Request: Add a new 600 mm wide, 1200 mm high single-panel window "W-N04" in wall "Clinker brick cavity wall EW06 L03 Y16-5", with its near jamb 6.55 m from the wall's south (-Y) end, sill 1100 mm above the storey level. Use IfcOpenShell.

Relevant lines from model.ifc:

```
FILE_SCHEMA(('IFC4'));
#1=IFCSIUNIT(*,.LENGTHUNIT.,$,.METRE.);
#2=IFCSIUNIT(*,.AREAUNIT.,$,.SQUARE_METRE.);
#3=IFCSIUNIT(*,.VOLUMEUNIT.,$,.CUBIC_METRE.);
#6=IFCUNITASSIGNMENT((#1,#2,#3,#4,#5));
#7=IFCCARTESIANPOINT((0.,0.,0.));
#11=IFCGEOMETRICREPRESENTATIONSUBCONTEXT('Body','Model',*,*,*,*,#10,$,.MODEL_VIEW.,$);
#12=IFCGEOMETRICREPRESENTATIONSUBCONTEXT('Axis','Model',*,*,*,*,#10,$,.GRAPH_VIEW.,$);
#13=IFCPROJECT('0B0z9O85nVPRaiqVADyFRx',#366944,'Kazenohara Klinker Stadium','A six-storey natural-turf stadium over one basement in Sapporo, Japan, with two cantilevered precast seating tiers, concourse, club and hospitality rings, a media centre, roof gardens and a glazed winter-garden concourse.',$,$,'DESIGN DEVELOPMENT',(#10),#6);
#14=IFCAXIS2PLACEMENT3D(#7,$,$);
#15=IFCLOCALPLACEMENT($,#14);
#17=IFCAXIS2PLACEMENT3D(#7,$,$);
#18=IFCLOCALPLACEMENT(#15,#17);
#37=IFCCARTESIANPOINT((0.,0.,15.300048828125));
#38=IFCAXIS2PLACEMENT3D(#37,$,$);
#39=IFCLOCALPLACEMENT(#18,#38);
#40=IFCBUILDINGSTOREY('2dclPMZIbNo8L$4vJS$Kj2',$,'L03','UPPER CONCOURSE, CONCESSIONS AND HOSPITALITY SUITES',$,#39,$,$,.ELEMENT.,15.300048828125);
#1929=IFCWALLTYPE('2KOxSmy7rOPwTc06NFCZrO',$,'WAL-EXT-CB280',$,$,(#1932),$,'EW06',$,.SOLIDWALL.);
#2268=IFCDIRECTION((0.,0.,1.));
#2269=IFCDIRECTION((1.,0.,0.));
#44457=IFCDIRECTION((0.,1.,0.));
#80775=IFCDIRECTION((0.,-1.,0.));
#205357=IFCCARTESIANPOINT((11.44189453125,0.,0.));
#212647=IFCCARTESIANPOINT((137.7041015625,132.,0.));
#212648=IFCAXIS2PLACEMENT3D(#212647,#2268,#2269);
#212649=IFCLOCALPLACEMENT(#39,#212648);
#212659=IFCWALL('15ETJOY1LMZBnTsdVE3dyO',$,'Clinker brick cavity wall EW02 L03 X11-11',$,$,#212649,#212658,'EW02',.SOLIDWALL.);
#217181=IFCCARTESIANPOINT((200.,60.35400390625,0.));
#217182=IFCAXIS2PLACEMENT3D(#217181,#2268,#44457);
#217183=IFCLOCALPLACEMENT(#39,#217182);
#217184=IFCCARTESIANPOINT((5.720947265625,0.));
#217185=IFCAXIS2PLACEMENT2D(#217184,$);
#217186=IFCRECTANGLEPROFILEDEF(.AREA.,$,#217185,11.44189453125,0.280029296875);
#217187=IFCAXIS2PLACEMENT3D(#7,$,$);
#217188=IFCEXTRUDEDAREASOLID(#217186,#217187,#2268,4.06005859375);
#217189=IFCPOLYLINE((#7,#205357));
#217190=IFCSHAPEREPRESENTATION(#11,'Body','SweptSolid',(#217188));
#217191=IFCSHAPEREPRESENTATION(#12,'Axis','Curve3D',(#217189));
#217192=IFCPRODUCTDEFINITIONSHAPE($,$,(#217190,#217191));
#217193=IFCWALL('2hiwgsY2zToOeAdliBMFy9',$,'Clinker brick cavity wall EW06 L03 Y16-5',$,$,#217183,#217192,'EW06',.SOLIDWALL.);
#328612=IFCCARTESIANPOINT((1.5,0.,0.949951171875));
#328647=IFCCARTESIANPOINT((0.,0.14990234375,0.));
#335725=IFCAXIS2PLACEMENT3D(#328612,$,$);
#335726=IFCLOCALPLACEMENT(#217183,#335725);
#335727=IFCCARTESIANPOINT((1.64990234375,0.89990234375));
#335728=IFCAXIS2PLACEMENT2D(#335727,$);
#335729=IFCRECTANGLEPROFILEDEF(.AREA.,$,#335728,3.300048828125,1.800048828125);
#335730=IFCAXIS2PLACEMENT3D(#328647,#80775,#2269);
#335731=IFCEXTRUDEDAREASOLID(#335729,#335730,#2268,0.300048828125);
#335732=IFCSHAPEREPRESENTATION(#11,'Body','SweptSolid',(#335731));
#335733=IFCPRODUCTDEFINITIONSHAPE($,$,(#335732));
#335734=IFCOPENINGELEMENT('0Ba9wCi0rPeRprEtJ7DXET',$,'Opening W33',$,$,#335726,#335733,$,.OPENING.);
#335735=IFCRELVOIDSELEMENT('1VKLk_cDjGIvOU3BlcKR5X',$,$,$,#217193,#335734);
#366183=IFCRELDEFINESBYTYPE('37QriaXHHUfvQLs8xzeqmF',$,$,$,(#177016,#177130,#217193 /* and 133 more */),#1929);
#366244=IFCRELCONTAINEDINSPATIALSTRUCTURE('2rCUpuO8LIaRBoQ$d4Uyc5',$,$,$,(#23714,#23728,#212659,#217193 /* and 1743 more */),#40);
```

```python
import numpy as np
import ifcopenshell
import ifcopenshell.api.feature
import ifcopenshell.api.geometry
import ifcopenshell.api.root
import ifcopenshell.api.spatial
import ifcopenshell.geom
import ifcopenshell.util.element
import ifcopenshell.util.placement
import ifcopenshell.util.representation
import ifcopenshell.util.shape
import ifcopenshell.util.unit

model = ifcopenshell.open("model.ifc")
unit_scale = ifcopenshell.util.unit.calculate_unit_scale(model)
settings = ifcopenshell.geom.settings()


def volume(element):
    """Net volume in cubic metres, openings subtracted."""
    shape = ifcopenshell.geom.create_shape(settings, element)
    return ifcopenshell.util.shape.get_volume(shape.geometry)


wall = model.by_guid("2hiwgsY2zToOeAdliBMFy9")
storey = ifcopenshell.util.element.get_container(wall, ifc_class="IfcBuildingStorey")
context = ifcopenshell.util.representation.get_context(model, "Model", "Body", "MODEL_VIEW")
before = volume(wall)

width, height, from_end, sill = 0.6, 1.2, 6.55, 1.1  # metres

# The wall runs along its own X axis, and the end named is its -X end.
wall_shape = ifcopenshell.geom.create_shape(settings, wall)
x, y, z = ifcopenshell.util.shape.get_vertices(wall_shape.geometry).T
start = x.min() + from_end
face, thickness = float(y.min()), float(y.max() - y.min())
wall_matrix = ifcopenshell.util.placement.get_local_placement(wall.ObjectPlacement)
level = ifcopenshell.util.placement.get_local_placement(storey.ObjectPlacement)[2, 3]


def in_wall(x, y):
    """Placement at x, y metres in the wall's axes, at sill height."""
    matrix = wall_matrix.copy()
    matrix[:, 3] = wall_matrix @ np.array([x / unit_scale, y / unit_scale, 0.0, 1.0])
    matrix[2, 3] = level + sill / unit_scale
    return matrix


# Opening: a box that overshoots both wall faces by 50 mm.
opening = ifcopenshell.api.root.create_entity(model, ifc_class="IfcOpeningElement", predefined_type="OPENING")
box = ifcopenshell.api.geometry.add_wall_representation(
    model, context=context, length=width, height=height, thickness=thickness + 0.1
)
ifcopenshell.api.geometry.assign_representation(model, product=opening, representation=box)
ifcopenshell.api.geometry.edit_object_placement(model, product=opening, matrix=in_wall(start, face - 0.05), is_si=False)
ifcopenshell.api.feature.add_feature(model, feature=opening, element=wall)

window = ifcopenshell.api.root.create_entity(model, ifc_class="IfcWindow", name="W-N04", predefined_type="WINDOW")
window.OverallWidth, window.OverallHeight = width / unit_scale, height / unit_scale
window.PartitioningType = "SINGLE_PANEL"
body = ifcopenshell.api.geometry.add_window_representation(
    model,
    context=context,
    overall_width=window.OverallWidth,
    overall_height=window.OverallHeight,
    partition_type="SINGLE_PANEL",
)
ifcopenshell.api.geometry.assign_representation(model, product=window, representation=body)
ifcopenshell.api.spatial.assign_container(model, products=[window], relating_structure=storey)
ifcopenshell.api.feature.add_filling(model, opening=opening, element=window)

# Centre the window in the wall's thickness.
ifcopenshell.api.geometry.edit_object_placement(model, product=window, matrix=in_wall(start, face), is_si=False)
window_shape = ifcopenshell.geom.create_shape(settings, window)
depth = ifcopenshell.util.shape.get_vertices(window_shape.geometry)[:, 1]
offset = face + thickness / 2 - (depth.min() + depth.max()) / 2
ifcopenshell.api.geometry.edit_object_placement(model, product=window, matrix=in_wall(start, offset), is_si=False)

after = volume(wall)

print(f"wall volume {before:.3f} -> {after:.3f} m3")

model.write("model_v2.ifc")
```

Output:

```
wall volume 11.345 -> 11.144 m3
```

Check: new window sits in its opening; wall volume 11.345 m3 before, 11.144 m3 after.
